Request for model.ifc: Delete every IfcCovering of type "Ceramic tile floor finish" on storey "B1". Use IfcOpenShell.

First a look at what the model holds.

```python
import ifcopenshell
import ifcopenshell.util.element

model = ifcopenshell.open("model.ifc")
print(model.schema)
storey = next(s for s in model.by_type("IfcBuildingStorey") if s.Name == "B1")
coverings = [e for e in ifcopenshell.util.element.get_decomposition(storey) if e.is_a("IfcCovering")]
seen = {}
for e in coverings:
    element_type = ifcopenshell.util.element.get_type(e)
    name = element_type.Name if element_type not in (None, e) else None
    seen[name] = seen.get(name, 0) + 1
for name, count in sorted(seen.items(), key=str):
    print(count, "x", name)
```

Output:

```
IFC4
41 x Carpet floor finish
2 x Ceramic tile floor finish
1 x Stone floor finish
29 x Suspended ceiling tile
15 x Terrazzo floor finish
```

```python
import ifcopenshell
import ifcopenshell.api.root
import ifcopenshell.util.element

model = ifcopenshell.open("model.ifc")

storey = next(s for s in model.by_type("IfcBuildingStorey") if s.Name == "B1")
coverings = [e for e in ifcopenshell.util.element.get_decomposition(storey) if e.is_a("IfcCovering")]
targets = [e for e in coverings if (t := ifcopenshell.util.element.get_type(e)) not in (None, e) and t.Name == "Ceramic tile floor finish"]

for e in targets:
    ifcopenshell.api.root.remove_product(model, product=e)
print(len(targets), "removed")

model.write("model_updated.ifc")
```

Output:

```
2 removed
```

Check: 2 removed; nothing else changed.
